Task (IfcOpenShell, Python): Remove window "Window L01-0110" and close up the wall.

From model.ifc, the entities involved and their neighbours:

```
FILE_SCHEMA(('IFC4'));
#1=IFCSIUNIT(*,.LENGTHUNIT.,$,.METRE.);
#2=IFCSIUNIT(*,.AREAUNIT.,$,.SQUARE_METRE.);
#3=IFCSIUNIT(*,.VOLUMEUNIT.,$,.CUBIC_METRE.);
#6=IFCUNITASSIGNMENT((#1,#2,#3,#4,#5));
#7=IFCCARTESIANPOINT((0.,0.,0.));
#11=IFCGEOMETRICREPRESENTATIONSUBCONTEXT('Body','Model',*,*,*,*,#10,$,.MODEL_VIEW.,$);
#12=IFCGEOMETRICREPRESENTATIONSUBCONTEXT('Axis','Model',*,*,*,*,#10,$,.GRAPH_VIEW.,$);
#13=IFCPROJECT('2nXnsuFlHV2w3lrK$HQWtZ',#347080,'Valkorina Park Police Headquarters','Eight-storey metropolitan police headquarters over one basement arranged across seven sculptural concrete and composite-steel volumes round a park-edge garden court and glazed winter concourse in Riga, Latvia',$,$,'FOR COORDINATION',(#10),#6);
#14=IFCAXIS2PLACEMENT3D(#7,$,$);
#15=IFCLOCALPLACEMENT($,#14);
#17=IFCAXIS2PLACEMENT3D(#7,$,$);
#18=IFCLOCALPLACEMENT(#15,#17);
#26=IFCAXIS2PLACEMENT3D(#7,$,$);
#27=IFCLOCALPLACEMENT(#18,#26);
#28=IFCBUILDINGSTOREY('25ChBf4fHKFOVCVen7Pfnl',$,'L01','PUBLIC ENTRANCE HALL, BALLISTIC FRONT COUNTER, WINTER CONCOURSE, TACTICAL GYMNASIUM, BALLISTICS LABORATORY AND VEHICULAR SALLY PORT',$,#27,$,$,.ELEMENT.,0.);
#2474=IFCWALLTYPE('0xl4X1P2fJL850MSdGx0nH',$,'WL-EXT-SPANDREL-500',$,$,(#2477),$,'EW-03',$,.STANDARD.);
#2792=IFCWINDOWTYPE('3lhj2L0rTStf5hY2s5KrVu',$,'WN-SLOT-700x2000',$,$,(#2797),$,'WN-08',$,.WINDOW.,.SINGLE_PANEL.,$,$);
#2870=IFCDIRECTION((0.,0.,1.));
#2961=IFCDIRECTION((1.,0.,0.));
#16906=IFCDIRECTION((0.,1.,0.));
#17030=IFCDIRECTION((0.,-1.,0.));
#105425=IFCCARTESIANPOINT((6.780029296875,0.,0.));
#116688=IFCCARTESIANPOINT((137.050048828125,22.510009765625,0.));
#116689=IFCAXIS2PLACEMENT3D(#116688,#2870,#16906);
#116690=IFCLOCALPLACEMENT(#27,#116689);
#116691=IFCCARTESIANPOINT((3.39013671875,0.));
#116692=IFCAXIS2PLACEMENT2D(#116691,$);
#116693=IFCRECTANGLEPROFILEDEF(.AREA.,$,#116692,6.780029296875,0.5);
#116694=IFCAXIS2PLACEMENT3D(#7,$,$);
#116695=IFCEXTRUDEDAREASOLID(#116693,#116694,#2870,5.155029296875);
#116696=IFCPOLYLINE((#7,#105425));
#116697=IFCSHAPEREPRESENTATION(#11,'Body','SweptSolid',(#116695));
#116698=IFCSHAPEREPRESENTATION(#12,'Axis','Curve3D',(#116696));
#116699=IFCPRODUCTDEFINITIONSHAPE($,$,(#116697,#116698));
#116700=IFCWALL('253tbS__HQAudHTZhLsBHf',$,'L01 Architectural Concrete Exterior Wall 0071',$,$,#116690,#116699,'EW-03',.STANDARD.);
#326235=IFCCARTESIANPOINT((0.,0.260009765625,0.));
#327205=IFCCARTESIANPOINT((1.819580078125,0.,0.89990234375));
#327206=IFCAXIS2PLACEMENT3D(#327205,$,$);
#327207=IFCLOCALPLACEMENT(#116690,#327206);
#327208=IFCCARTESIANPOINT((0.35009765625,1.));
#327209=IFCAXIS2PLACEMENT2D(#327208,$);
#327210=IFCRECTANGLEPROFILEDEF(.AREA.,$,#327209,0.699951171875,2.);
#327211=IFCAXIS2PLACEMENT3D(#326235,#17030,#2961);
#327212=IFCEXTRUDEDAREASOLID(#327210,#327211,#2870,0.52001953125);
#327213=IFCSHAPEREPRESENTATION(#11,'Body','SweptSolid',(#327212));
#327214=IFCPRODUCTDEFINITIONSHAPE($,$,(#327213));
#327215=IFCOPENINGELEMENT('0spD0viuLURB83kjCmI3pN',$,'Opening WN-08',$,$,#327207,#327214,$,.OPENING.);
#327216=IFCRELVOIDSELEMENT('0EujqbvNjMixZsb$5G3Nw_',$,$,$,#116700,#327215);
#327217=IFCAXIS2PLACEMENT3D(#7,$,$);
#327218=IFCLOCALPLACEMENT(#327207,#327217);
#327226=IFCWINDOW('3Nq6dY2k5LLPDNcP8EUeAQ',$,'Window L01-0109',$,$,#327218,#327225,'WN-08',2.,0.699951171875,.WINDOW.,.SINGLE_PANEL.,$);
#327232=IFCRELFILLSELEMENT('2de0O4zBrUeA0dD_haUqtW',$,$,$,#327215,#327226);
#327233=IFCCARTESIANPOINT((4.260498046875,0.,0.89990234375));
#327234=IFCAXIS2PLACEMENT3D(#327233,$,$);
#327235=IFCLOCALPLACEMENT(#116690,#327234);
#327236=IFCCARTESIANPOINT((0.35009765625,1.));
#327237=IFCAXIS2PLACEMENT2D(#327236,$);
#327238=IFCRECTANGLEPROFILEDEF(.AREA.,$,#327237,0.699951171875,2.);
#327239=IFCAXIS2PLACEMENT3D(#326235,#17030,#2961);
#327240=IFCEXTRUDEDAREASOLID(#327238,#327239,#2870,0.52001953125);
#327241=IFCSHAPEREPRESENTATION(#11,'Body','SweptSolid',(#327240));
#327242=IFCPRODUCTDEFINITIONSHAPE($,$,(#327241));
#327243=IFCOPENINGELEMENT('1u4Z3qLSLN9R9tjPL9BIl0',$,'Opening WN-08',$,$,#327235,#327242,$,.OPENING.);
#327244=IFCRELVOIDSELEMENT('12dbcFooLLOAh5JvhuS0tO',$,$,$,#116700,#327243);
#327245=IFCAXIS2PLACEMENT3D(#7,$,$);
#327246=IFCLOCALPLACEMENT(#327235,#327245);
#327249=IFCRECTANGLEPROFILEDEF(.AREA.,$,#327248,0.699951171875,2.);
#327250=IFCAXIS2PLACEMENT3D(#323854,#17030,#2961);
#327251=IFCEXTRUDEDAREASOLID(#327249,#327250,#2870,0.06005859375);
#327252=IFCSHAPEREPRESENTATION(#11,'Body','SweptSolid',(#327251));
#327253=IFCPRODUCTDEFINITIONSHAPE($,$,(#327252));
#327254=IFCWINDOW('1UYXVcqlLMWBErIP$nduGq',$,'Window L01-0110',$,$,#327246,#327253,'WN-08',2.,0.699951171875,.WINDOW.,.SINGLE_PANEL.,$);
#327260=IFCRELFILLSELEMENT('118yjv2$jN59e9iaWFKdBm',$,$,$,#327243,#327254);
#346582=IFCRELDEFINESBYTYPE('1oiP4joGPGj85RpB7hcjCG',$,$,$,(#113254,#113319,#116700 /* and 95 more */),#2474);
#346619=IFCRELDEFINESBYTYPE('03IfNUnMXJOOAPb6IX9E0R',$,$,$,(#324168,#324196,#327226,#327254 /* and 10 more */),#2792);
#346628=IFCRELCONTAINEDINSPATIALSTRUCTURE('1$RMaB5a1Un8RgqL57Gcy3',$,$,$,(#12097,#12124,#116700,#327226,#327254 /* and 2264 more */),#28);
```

```python
import ifcopenshell
import ifcopenshell.api.feature
import ifcopenshell.api.root
import ifcopenshell.geom
import ifcopenshell.util.shape

model = ifcopenshell.open("model.ifc")
settings = ifcopenshell.geom.settings()


def volume(element):
    """Net volume in cubic metres, openings subtracted."""
    shape = ifcopenshell.geom.create_shape(settings, element)
    return ifcopenshell.util.shape.get_volume(shape.geometry)


window = model.by_guid("1UYXVcqlLMWBErIP$nduGq")
opening = window.FillsVoids[0].RelatingOpeningElement
wall = opening.VoidsElements[0].RelatingBuildingElement
before = volume(wall)

ifcopenshell.api.root.remove_product(model, product=window)
ifcopenshell.api.feature.remove_feature(model, feature=opening)

after = volume(wall)

print(f"wall volume {before:.3f} -> {after:.3f} m3")

model.write("model_rev.ifc")
```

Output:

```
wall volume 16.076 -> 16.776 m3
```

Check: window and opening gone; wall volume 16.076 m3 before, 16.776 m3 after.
